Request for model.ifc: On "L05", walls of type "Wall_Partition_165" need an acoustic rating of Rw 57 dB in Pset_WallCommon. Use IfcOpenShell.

First a look at what the model holds.

```python
import ifcopenshell
import ifcopenshell.util.element

model = ifcopenshell.open("model.ifc")
print(model.schema)
storey = next(s for s in model.by_type("IfcBuildingStorey") if s.Name == "L05")
walls = [e for e in ifcopenshell.util.element.get_decomposition(storey) if e.is_a("IfcWall")]
seen = {}
for e in walls:
    element_type = ifcopenshell.util.element.get_type(e)
    key = (element_type.Name if element_type != e and element_type else None, ifcopenshell.util.element.get_pset(e, "Pset_WallCommon", "AcousticRating"))
    seen[key] = seen.get(key, 0) + 1
for (name, value), count in sorted(seen.items(), key=str):
    print(count, "x", name, "|", value)
```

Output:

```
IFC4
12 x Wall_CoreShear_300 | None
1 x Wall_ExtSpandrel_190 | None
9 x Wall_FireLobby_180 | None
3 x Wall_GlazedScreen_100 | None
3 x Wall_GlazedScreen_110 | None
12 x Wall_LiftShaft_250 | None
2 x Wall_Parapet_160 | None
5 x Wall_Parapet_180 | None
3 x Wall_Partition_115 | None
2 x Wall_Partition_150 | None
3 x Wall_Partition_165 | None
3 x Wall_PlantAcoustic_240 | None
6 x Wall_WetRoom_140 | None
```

```python
import ifcopenshell
import ifcopenshell.api.pset
import ifcopenshell.util.element

model = ifcopenshell.open("model.ifc")

storey = next(s for s in model.by_type("IfcBuildingStorey") if s.Name == "L05")
walls = [e for e in ifcopenshell.util.element.get_decomposition(storey) if e.is_a("IfcWall")]

count = 0
for e in walls:
    element_type = ifcopenshell.util.element.get_type(e)
    if element_type in (None, e) or element_type.Name != "Wall_Partition_165":
        continue
    # add_pset returns the element's existing set when there is one.
    pset = ifcopenshell.api.pset.add_pset(model, product=e, name="Pset_WallCommon")
    ifcopenshell.api.pset.edit_pset(model, pset=pset, properties={"AcousticRating": "Rw 57 dB"})
    count += 1

print(count, "walls updated")

model.write("model_edited.ifc")
```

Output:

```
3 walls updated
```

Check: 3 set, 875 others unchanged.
